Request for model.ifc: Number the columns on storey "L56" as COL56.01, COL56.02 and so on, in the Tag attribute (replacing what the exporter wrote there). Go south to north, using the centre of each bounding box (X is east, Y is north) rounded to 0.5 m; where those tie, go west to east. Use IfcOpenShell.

First a look at what the model holds.

```python
import ifcopenshell
import ifcopenshell.util.element
import ifcopenshell.util.placement

model = ifcopenshell.open("model.ifc")
print(model.schema)
storey = next(s for s in model.by_type("IfcBuildingStorey") if s.Name == "L56")
columns = [e for e in ifcopenshell.util.element.get_decomposition(storey) if e.is_a("IfcColumn")]
for e in sorted(columns, key=lambda e: e.id()):
    origin = ifcopenshell.util.placement.get_local_placement(e.ObjectPlacement)[:3, 3]
    print(e.id(), e.Tag, e.Name, origin.round(2) + 0.0, sep=" | ")
```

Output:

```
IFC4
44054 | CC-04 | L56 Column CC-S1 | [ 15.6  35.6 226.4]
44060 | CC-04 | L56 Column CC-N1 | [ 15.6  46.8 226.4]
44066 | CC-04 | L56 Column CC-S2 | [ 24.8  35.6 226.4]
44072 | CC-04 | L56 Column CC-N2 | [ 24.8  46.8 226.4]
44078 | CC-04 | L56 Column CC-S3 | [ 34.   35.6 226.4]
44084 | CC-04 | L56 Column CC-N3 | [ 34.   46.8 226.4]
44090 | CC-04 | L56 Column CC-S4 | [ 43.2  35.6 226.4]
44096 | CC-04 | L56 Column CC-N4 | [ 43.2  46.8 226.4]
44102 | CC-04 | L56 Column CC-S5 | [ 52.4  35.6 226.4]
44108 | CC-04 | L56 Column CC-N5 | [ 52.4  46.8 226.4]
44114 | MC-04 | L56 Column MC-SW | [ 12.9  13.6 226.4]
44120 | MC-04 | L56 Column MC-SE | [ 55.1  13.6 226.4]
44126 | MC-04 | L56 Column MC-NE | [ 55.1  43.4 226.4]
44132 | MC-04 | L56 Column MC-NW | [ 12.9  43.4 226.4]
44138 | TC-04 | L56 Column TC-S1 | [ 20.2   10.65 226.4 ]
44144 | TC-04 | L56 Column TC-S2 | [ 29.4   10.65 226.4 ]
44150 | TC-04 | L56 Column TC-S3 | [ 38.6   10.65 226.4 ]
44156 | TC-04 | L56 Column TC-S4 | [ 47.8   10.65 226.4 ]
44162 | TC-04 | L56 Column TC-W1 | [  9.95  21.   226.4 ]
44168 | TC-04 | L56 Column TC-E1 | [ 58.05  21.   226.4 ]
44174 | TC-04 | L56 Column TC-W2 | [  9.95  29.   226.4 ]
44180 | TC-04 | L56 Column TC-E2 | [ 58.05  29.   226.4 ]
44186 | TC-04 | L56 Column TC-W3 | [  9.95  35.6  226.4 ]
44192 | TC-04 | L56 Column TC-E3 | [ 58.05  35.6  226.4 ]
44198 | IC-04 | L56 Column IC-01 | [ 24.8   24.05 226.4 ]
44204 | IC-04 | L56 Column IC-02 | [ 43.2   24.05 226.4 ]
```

```python
import ifcopenshell
import ifcopenshell.geom
import ifcopenshell.util.element
import ifcopenshell.util.shape

model = ifcopenshell.open("model.ifc")
settings = ifcopenshell.geom.settings()
settings.set("use-world-coords", True)


def centre(element):
    shape = ifcopenshell.geom.create_shape(settings, element)
    return ifcopenshell.util.shape.get_bbox_centroid(shape.geometry)


storey = next(s for s in model.by_type("IfcBuildingStorey") if s.Name == "L56")
columns = [e for e in ifcopenshell.util.element.get_decomposition(storey) if e.is_a("IfcColumn")]

# Insertion points can sit at a corner or the storey origin, so sort by the geometry (in metres).
centres = {e: centre(e) for e in columns}
columns.sort(key=lambda e: (round(centres[e][1] / 0.5), centres[e][0]))

for i, e in enumerate(columns, start=1):
    number = f"COL56.{i:02d}"
    e.Tag = number
    print(e.id(), number)

model.write("model-out.ifc")
```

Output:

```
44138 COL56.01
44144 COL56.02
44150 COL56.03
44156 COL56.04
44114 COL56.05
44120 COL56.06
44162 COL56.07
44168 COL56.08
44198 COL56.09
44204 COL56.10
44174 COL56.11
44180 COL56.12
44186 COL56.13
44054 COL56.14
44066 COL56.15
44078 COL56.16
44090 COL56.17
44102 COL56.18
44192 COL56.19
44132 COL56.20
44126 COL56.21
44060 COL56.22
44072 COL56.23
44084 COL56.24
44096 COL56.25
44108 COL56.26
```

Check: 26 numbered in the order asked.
